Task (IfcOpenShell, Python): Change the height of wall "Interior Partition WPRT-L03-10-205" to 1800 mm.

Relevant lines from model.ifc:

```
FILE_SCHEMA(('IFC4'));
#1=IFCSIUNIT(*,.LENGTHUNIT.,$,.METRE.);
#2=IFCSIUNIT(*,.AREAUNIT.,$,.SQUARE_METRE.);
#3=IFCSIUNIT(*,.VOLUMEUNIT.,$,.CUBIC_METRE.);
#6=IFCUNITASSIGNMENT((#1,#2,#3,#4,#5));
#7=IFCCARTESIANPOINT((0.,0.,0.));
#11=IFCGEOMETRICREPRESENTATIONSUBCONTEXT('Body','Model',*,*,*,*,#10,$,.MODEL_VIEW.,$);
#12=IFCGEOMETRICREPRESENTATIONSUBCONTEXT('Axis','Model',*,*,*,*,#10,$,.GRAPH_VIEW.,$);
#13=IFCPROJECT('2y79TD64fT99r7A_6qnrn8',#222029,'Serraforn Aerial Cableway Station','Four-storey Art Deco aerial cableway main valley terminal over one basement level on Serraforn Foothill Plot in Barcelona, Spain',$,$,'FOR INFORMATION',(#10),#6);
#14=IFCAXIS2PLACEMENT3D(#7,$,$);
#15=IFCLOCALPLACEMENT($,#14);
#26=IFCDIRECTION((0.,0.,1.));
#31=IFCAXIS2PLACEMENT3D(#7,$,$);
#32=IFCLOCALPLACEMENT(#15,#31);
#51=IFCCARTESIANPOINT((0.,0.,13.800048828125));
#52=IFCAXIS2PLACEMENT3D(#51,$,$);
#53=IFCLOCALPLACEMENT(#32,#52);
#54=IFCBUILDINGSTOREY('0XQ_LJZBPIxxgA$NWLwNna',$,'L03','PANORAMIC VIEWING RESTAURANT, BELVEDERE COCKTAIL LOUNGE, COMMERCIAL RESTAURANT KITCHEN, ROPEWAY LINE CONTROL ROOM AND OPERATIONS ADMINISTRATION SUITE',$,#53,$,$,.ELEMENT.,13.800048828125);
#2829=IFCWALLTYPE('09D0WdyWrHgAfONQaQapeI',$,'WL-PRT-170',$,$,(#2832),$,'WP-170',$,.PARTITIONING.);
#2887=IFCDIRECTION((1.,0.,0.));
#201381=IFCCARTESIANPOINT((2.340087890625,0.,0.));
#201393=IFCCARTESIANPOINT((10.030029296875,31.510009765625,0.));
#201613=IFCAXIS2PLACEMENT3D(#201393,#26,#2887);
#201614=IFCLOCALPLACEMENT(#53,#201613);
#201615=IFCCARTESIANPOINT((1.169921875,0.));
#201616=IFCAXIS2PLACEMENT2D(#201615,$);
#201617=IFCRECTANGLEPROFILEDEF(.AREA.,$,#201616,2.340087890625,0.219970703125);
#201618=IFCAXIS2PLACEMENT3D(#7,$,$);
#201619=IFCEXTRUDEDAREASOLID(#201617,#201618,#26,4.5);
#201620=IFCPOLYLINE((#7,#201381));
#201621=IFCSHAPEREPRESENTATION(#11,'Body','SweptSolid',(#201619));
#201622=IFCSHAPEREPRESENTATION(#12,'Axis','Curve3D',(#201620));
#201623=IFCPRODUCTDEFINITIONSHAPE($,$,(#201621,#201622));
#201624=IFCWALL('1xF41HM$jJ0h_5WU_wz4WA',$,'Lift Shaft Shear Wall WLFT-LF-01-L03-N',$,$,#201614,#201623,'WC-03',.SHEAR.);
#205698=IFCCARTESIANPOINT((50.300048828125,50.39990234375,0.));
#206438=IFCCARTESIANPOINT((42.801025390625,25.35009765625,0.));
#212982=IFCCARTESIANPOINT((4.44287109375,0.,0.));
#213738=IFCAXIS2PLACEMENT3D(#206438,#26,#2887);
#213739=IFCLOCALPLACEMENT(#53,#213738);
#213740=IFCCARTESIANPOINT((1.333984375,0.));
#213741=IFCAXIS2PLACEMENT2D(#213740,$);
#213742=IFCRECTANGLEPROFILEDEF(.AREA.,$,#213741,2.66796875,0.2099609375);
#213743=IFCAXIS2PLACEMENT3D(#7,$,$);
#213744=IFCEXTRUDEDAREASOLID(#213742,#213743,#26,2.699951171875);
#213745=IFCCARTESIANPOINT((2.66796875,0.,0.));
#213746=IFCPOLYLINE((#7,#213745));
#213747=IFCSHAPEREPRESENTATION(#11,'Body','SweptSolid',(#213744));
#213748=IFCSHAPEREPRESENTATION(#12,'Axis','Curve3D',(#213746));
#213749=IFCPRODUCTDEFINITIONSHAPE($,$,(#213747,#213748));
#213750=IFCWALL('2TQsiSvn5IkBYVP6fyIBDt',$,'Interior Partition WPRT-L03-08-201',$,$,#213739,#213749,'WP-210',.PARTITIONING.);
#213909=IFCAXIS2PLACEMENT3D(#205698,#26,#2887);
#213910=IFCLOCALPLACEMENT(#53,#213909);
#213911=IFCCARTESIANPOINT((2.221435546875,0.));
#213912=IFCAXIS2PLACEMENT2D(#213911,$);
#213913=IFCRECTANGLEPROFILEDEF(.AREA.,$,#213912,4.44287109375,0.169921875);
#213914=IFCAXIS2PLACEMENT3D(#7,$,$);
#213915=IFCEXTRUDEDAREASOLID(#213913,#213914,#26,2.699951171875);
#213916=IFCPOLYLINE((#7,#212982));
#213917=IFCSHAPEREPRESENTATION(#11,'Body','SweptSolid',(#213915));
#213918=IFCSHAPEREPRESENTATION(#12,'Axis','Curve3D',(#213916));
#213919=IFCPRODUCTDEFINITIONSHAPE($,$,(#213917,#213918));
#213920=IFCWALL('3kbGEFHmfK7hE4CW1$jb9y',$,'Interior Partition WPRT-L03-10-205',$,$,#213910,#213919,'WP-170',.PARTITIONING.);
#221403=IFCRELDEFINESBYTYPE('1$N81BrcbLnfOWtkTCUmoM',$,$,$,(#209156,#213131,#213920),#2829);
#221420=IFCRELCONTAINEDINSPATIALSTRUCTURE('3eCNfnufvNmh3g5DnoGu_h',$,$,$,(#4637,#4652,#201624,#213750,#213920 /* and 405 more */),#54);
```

```python
import ifcopenshell
import ifcopenshell.geom
import ifcopenshell.util.representation
import ifcopenshell.util.shape

model = ifcopenshell.open("model.ifc")
settings = ifcopenshell.geom.settings()


def volume(element):
    """Net volume in cubic metres, openings subtracted."""
    shape = ifcopenshell.geom.create_shape(settings, element)
    return ifcopenshell.util.shape.get_volume(shape.geometry)


wall = model.by_guid("3kbGEFHmfK7hE4CW1$jb9y")
before = volume(wall)

body = ifcopenshell.util.representation.get_representation(wall, "Model", "Body")
solid = body.Items[0]
old_height = solid.Depth
solid.Depth = 1.8
after = volume(wall)

print(f"height {old_height:g} -> {solid.Depth:g}, volume {before:.3f} -> {after:.3f} m3")

model.write("model_updated.ifc")
```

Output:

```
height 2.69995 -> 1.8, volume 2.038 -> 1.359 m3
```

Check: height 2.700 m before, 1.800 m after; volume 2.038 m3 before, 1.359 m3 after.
